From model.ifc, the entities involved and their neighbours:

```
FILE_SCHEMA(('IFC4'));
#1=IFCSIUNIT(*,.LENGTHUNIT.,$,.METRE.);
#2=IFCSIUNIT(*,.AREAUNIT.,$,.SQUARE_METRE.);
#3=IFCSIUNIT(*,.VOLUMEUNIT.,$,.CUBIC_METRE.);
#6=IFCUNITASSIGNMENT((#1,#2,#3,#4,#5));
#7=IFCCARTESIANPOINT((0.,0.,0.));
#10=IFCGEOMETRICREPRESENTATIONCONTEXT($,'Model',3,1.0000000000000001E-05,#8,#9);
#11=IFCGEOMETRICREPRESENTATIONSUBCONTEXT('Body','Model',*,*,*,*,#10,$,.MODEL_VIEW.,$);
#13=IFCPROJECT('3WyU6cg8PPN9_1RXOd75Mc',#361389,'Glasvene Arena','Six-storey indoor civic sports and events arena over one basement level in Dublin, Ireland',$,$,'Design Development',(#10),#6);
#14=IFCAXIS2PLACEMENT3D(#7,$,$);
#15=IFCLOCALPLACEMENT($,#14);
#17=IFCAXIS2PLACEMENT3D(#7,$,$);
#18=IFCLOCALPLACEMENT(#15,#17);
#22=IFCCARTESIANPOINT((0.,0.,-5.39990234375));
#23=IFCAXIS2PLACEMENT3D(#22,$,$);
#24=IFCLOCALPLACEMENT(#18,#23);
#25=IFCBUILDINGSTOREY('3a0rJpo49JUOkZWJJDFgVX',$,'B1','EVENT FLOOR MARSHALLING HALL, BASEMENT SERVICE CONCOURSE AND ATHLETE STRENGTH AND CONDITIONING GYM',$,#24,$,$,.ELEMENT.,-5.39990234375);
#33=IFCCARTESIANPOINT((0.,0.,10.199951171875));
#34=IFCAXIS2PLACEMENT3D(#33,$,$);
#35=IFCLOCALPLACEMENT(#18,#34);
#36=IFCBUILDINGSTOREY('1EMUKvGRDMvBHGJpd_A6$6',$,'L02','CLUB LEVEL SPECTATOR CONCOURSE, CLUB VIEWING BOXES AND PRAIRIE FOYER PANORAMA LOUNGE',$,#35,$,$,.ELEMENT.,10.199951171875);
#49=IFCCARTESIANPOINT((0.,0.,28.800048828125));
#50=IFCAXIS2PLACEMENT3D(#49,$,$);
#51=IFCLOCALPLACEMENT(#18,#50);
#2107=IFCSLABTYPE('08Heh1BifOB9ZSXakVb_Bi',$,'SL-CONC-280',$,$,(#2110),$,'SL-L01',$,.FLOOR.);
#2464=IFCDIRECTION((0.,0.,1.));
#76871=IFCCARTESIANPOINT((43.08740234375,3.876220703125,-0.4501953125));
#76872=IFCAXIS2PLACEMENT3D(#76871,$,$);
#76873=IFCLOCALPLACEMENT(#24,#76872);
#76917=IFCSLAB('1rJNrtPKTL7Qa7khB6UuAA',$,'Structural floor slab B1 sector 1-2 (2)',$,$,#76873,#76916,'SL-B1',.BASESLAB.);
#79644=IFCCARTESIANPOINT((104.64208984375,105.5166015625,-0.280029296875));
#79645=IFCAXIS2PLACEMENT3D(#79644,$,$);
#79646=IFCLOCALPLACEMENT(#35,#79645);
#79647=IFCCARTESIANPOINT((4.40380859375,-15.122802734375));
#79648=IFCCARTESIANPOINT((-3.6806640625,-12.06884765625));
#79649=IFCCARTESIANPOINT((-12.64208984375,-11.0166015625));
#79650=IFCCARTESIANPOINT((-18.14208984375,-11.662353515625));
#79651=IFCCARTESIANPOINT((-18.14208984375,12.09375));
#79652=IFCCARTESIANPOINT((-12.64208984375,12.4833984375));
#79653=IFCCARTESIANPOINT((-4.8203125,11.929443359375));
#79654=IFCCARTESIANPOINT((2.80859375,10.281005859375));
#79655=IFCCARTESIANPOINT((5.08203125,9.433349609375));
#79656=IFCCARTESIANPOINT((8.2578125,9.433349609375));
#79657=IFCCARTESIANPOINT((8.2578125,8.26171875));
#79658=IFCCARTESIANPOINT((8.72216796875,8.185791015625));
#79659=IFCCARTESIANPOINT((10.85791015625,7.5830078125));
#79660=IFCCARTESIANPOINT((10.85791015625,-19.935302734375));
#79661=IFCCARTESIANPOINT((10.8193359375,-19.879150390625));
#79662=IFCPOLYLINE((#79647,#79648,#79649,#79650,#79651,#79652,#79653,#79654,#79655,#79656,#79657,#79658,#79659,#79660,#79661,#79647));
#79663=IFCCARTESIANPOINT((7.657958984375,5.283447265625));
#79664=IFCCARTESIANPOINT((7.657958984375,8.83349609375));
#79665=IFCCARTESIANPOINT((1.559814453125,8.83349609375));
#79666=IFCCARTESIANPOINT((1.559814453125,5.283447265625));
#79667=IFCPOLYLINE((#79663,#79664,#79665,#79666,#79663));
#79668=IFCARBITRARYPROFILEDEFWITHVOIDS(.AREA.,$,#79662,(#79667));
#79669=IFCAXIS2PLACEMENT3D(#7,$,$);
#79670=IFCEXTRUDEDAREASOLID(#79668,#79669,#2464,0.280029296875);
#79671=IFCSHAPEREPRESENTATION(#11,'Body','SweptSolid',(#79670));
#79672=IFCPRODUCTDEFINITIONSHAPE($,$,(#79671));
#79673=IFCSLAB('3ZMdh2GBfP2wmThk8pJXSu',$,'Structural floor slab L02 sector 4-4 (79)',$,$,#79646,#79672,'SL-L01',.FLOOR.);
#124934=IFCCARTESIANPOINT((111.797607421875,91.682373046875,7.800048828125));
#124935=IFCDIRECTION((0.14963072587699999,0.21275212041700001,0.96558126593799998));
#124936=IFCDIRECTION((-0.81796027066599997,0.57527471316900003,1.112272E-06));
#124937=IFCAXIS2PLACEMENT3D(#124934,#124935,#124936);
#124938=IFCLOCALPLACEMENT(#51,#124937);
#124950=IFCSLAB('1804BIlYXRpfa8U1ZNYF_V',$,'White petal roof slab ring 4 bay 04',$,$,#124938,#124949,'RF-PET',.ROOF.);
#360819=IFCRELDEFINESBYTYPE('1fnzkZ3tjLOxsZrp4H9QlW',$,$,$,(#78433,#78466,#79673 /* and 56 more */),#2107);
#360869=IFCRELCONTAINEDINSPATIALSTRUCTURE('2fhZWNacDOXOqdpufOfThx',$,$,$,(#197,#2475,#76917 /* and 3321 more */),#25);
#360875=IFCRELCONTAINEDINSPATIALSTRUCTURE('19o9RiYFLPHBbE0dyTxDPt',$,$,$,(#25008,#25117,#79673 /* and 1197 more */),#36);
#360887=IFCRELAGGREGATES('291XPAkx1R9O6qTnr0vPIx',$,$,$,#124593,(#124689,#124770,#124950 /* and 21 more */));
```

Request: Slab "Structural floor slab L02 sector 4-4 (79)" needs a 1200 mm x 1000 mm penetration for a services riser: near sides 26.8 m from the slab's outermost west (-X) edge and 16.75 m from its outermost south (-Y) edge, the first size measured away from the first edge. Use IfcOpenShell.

```python
import numpy as np
import ifcopenshell
import ifcopenshell.api.feature
import ifcopenshell.api.geometry
import ifcopenshell.api.root
import ifcopenshell.geom
import ifcopenshell.util.placement
import ifcopenshell.util.representation
import ifcopenshell.util.shape
import ifcopenshell.util.unit

model = ifcopenshell.open("model.ifc")
unit_scale = ifcopenshell.util.unit.calculate_unit_scale(model)
settings = ifcopenshell.geom.settings()


def volume(element):
    """Net volume in cubic metres, openings subtracted."""
    shape = ifcopenshell.geom.create_shape(settings, element)
    return ifcopenshell.util.shape.get_volume(shape.geometry)


slab = model.by_guid("3ZMdh2GBfP2wmThk8pJXSu")
before = volume(slab)

# Extent in the slab's own axes, in metres. The edges named are its -X and -Y sides.
slab_shape = ifcopenshell.geom.create_shape(settings, slab)
vertices = ifcopenshell.util.shape.get_vertices(slab_shape.geometry)
x_min, y_min, bottom = vertices.min(axis=0)
top = vertices[:, 2].max()

opening = ifcopenshell.api.root.create_entity(model, ifc_class="IfcOpeningElement", name="Services riser opening", predefined_type="OPENING")
context = ifcopenshell.util.representation.get_context(model, "Model", "Body", "MODEL_VIEW")
width, depth = 1.2, 1
outline = [(0.0, 0.0), (width, 0.0), (width, depth), (0.0, depth), (0.0, 0.0)]
# Overshoot both faces by 50 mm so the cut is clean.
shape = ifcopenshell.api.geometry.add_slab_representation(
    model, context=context, depth=top - bottom + 0.1, polyline=outline
)
ifcopenshell.api.geometry.assign_representation(model, product=opening, representation=shape)

matrix = ifcopenshell.util.placement.get_local_placement(slab.ObjectPlacement)
matrix[:, 3] = matrix @ np.append(np.array([x_min + 26.8, y_min + 16.75, bottom - 0.05]) / unit_scale, 1.0)
ifcopenshell.api.geometry.edit_object_placement(model, product=opening, matrix=matrix, is_si=False)
ifcopenshell.api.feature.add_feature(model, feature=opening, element=slab)

after = volume(slab)

print(f"slab volume {before:.3f} -> {after:.3f} m3")

model.write("model-out.ifc")
```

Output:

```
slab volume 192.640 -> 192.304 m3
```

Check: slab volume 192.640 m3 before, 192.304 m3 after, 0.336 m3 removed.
